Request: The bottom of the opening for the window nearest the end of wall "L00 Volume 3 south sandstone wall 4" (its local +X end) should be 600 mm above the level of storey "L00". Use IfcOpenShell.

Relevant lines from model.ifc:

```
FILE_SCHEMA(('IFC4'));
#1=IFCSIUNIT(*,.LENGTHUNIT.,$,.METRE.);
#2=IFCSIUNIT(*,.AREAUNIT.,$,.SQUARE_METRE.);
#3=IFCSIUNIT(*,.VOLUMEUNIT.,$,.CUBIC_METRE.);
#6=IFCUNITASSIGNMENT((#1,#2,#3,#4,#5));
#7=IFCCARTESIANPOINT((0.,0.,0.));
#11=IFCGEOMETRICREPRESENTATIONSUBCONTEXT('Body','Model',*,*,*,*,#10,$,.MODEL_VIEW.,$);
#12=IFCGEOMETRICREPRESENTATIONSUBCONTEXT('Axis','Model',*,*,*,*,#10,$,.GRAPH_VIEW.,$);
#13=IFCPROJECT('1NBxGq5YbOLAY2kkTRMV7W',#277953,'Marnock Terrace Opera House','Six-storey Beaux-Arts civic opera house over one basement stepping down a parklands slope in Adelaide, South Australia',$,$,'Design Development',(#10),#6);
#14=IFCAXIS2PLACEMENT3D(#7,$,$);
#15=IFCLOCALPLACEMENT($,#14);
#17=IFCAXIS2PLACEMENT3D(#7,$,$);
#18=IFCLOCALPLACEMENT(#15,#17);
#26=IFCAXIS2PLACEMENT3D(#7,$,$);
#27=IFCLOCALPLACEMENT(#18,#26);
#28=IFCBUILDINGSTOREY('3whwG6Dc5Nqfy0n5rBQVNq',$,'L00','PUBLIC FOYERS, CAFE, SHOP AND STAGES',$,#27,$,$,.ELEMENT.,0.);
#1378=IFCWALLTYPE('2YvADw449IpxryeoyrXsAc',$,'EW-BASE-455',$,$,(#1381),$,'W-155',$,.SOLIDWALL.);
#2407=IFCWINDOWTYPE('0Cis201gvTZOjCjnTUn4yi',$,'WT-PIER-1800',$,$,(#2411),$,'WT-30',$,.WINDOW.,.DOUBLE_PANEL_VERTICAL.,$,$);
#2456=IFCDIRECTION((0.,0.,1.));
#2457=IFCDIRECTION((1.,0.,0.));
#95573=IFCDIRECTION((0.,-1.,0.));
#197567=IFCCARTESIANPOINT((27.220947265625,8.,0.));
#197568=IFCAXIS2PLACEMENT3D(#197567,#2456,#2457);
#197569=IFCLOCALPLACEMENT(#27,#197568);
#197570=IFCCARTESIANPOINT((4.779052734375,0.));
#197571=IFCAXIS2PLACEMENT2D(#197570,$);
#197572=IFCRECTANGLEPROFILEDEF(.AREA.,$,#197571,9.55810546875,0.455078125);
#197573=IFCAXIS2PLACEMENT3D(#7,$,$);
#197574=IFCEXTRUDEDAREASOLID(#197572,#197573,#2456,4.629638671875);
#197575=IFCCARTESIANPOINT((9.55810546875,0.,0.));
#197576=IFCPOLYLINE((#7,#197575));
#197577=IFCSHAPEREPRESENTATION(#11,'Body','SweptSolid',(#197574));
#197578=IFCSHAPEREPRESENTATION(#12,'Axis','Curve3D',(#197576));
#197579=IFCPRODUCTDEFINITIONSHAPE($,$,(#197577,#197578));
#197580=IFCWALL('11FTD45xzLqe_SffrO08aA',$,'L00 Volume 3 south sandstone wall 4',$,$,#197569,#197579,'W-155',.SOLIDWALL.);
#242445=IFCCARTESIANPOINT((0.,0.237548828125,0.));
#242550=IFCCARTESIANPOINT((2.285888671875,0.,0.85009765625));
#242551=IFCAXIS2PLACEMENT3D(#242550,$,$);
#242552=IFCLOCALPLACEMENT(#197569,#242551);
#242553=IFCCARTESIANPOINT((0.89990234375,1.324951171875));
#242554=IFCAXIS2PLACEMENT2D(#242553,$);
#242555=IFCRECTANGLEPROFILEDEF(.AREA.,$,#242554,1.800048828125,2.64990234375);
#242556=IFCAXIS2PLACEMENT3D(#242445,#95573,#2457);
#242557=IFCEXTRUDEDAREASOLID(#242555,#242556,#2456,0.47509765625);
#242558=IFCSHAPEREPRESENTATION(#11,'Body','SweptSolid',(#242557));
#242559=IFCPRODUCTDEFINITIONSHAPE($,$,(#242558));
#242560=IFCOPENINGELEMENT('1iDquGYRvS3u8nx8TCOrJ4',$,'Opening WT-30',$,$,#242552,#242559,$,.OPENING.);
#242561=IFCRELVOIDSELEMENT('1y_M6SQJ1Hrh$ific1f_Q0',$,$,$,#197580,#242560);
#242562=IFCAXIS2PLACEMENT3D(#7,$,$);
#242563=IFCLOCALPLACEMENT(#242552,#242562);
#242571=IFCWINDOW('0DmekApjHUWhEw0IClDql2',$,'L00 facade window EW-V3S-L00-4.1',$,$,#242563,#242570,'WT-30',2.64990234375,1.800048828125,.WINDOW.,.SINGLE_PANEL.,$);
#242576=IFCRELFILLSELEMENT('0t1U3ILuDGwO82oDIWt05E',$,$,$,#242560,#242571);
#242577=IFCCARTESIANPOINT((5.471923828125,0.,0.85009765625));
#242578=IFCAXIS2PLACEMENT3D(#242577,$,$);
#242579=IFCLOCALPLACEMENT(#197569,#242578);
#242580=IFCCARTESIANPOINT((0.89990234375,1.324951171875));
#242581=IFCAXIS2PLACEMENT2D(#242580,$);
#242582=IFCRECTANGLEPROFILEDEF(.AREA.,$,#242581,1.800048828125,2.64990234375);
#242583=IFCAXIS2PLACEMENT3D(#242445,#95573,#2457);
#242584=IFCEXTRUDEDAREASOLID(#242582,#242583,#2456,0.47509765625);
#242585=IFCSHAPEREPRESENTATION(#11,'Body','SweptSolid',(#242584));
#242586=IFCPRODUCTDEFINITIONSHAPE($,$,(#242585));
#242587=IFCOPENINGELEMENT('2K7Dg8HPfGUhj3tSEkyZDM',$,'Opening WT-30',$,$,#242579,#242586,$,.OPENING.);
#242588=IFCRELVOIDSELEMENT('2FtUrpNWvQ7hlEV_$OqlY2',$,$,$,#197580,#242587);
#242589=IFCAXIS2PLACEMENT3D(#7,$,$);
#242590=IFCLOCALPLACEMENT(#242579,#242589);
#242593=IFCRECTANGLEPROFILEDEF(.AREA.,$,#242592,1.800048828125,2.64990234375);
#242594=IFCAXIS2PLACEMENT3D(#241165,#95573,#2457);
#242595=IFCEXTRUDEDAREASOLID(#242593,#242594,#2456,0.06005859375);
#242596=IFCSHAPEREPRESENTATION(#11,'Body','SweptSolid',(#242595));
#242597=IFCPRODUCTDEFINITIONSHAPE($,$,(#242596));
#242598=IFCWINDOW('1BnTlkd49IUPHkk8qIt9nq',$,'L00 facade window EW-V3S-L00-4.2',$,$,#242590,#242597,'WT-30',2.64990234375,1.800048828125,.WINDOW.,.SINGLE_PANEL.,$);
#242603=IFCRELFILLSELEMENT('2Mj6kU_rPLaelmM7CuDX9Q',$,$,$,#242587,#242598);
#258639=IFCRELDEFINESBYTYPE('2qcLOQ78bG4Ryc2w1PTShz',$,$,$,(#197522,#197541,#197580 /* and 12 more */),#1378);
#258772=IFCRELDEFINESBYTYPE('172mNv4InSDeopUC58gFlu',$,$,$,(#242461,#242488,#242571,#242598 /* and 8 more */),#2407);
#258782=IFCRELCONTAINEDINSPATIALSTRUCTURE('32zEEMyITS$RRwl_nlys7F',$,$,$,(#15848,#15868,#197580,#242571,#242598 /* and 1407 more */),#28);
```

```python
import numpy as np
import ifcopenshell
import ifcopenshell.api.geometry
import ifcopenshell.geom
import ifcopenshell.util.element
import ifcopenshell.util.placement
import ifcopenshell.util.shape
import ifcopenshell.util.unit

model = ifcopenshell.open("model.ifc")
unit_scale = ifcopenshell.util.unit.calculate_unit_scale(model)

window = model.by_guid("1BnTlkd49IUPHkk8qIt9nq")
opening = window.FillsVoids[0].RelatingOpeningElement
storey = ifcopenshell.util.element.get_container(window, ifc_class="IfcBuildingStorey")
level = ifcopenshell.util.placement.get_local_placement(storey.ObjectPlacement)[2, 3]

# The opening's origin need not be at the sill, so measure its lowest point.
shape = ifcopenshell.geom.create_shape(ifcopenshell.geom.settings(), opening)
bottom = ifcopenshell.util.shape.get_shape_bottom_elevation(shape, shape.geometry) / unit_scale
dz = level + 0.6 / unit_scale - bottom

shift = np.array([0.0, 0.0, dz])
# The window is placed relative to its opening, so it follows when the opening moves.
matrix = ifcopenshell.util.placement.get_local_placement(opening.ObjectPlacement)
matrix[:3, 3] += shift
ifcopenshell.api.geometry.edit_object_placement(
    model, product=opening, matrix=matrix, is_si=False, should_transform_children=True
)

print(f"moved by {dz * unit_scale:+.3f} m")

model.write("model_edited.ifc")
```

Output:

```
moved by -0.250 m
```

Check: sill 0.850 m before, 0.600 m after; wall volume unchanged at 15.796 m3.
